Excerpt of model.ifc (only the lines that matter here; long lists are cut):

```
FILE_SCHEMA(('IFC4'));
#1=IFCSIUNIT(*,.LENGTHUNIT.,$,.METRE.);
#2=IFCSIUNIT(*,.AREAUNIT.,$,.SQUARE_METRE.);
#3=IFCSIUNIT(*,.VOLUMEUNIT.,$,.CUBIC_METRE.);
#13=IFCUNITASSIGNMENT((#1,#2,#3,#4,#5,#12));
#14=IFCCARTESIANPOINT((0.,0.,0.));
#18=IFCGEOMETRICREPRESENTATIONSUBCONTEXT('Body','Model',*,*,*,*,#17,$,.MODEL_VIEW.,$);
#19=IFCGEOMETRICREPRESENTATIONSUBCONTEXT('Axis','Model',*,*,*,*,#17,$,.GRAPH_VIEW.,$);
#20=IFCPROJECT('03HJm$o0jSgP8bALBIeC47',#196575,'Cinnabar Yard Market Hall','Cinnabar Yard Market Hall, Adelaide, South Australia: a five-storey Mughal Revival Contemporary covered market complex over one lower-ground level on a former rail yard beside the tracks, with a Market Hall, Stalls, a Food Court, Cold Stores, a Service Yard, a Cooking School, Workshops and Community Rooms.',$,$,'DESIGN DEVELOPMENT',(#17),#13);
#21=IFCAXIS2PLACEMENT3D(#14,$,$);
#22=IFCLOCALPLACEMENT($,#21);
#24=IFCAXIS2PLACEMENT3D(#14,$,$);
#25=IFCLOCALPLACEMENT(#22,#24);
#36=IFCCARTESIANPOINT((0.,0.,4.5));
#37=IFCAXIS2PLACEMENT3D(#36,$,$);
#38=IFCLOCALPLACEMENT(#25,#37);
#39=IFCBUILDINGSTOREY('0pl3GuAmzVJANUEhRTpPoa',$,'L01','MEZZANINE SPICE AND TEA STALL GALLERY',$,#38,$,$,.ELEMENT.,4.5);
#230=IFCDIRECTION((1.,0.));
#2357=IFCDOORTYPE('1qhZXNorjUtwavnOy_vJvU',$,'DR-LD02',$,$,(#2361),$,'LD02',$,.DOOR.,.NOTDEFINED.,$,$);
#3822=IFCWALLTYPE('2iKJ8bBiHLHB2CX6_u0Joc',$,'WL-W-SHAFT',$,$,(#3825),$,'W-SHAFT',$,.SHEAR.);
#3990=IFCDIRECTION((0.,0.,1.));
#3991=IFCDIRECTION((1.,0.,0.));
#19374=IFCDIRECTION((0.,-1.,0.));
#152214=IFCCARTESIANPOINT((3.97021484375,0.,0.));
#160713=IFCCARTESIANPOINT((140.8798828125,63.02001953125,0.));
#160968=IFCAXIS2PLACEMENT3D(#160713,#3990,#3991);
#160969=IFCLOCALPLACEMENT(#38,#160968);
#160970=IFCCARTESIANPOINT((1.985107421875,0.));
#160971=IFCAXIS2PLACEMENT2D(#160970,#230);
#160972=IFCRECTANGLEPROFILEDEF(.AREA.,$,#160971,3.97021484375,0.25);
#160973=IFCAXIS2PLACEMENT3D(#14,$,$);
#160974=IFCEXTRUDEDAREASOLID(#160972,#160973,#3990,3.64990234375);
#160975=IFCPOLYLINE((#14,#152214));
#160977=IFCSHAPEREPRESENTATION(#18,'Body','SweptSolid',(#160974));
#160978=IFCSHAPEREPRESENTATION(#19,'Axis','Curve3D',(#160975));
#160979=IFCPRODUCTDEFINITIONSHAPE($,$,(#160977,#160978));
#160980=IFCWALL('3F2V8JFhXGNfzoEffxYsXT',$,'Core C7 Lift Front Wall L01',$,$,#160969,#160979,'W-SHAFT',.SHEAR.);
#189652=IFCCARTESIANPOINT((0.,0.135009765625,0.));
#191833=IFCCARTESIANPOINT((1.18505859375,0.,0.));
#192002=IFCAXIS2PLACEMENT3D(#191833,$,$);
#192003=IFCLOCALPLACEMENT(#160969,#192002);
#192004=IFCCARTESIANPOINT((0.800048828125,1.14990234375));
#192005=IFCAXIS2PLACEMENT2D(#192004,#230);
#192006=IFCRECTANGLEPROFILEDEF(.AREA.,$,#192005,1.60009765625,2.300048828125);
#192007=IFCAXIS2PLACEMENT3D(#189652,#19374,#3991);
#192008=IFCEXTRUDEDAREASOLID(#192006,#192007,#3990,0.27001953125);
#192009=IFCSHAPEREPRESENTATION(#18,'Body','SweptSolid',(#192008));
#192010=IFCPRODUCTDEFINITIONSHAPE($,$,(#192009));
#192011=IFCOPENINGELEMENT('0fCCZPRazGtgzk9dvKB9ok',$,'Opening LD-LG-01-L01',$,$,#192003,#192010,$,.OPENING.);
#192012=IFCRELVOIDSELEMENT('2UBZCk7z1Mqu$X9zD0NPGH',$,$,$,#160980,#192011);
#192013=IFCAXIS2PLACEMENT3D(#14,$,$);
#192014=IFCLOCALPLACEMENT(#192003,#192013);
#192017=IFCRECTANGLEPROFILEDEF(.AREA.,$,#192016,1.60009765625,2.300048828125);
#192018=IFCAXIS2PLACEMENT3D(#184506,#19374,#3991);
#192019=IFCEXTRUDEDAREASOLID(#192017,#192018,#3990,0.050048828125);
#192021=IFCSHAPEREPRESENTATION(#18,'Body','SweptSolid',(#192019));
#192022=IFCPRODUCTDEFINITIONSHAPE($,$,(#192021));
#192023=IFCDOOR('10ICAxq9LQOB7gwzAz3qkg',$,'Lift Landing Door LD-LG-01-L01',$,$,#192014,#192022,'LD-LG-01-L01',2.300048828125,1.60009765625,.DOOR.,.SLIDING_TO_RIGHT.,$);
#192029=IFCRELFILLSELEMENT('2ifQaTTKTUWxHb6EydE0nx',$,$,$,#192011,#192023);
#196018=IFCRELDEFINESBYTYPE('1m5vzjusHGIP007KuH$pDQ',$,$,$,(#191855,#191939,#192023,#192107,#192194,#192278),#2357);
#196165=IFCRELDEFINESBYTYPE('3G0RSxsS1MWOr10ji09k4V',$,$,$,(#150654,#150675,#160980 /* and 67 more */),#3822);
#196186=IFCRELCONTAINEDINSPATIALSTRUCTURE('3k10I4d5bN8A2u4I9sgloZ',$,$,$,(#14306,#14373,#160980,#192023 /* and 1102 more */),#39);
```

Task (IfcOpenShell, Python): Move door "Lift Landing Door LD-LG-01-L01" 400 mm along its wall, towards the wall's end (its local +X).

```python
import ifcopenshell
import ifcopenshell.api.geometry
import ifcopenshell.util.placement
import ifcopenshell.util.unit

model = ifcopenshell.open("model.ifc")
unit_scale = ifcopenshell.util.unit.calculate_unit_scale(model)

door = model.by_guid("10ICAxq9LQOB7gwzAz3qkg")
opening = door.FillsVoids[0].RelatingOpeningElement
wall = opening.VoidsElements[0].RelatingBuildingElement

wall_matrix = ifcopenshell.util.placement.get_local_placement(wall.ObjectPlacement)
shift = wall_matrix[:3, 0] * 0.4 / unit_scale
before = ifcopenshell.util.placement.get_local_placement(door.ObjectPlacement)[:3, 3].copy()

# The door is placed relative to its opening, so it follows when the opening moves.
matrix = ifcopenshell.util.placement.get_local_placement(opening.ObjectPlacement)
matrix[:3, 3] += shift
ifcopenshell.api.geometry.edit_object_placement(
    model, product=opening, matrix=matrix, is_si=False, should_transform_children=True
)

after = ifcopenshell.util.placement.get_local_placement(door.ObjectPlacement)[:3, 3]
print("door moved by", (after - before).round(3) + 0.0)

model.write("model_edited.ifc")
```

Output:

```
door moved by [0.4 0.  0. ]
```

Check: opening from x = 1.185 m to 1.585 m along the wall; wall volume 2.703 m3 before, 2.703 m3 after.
